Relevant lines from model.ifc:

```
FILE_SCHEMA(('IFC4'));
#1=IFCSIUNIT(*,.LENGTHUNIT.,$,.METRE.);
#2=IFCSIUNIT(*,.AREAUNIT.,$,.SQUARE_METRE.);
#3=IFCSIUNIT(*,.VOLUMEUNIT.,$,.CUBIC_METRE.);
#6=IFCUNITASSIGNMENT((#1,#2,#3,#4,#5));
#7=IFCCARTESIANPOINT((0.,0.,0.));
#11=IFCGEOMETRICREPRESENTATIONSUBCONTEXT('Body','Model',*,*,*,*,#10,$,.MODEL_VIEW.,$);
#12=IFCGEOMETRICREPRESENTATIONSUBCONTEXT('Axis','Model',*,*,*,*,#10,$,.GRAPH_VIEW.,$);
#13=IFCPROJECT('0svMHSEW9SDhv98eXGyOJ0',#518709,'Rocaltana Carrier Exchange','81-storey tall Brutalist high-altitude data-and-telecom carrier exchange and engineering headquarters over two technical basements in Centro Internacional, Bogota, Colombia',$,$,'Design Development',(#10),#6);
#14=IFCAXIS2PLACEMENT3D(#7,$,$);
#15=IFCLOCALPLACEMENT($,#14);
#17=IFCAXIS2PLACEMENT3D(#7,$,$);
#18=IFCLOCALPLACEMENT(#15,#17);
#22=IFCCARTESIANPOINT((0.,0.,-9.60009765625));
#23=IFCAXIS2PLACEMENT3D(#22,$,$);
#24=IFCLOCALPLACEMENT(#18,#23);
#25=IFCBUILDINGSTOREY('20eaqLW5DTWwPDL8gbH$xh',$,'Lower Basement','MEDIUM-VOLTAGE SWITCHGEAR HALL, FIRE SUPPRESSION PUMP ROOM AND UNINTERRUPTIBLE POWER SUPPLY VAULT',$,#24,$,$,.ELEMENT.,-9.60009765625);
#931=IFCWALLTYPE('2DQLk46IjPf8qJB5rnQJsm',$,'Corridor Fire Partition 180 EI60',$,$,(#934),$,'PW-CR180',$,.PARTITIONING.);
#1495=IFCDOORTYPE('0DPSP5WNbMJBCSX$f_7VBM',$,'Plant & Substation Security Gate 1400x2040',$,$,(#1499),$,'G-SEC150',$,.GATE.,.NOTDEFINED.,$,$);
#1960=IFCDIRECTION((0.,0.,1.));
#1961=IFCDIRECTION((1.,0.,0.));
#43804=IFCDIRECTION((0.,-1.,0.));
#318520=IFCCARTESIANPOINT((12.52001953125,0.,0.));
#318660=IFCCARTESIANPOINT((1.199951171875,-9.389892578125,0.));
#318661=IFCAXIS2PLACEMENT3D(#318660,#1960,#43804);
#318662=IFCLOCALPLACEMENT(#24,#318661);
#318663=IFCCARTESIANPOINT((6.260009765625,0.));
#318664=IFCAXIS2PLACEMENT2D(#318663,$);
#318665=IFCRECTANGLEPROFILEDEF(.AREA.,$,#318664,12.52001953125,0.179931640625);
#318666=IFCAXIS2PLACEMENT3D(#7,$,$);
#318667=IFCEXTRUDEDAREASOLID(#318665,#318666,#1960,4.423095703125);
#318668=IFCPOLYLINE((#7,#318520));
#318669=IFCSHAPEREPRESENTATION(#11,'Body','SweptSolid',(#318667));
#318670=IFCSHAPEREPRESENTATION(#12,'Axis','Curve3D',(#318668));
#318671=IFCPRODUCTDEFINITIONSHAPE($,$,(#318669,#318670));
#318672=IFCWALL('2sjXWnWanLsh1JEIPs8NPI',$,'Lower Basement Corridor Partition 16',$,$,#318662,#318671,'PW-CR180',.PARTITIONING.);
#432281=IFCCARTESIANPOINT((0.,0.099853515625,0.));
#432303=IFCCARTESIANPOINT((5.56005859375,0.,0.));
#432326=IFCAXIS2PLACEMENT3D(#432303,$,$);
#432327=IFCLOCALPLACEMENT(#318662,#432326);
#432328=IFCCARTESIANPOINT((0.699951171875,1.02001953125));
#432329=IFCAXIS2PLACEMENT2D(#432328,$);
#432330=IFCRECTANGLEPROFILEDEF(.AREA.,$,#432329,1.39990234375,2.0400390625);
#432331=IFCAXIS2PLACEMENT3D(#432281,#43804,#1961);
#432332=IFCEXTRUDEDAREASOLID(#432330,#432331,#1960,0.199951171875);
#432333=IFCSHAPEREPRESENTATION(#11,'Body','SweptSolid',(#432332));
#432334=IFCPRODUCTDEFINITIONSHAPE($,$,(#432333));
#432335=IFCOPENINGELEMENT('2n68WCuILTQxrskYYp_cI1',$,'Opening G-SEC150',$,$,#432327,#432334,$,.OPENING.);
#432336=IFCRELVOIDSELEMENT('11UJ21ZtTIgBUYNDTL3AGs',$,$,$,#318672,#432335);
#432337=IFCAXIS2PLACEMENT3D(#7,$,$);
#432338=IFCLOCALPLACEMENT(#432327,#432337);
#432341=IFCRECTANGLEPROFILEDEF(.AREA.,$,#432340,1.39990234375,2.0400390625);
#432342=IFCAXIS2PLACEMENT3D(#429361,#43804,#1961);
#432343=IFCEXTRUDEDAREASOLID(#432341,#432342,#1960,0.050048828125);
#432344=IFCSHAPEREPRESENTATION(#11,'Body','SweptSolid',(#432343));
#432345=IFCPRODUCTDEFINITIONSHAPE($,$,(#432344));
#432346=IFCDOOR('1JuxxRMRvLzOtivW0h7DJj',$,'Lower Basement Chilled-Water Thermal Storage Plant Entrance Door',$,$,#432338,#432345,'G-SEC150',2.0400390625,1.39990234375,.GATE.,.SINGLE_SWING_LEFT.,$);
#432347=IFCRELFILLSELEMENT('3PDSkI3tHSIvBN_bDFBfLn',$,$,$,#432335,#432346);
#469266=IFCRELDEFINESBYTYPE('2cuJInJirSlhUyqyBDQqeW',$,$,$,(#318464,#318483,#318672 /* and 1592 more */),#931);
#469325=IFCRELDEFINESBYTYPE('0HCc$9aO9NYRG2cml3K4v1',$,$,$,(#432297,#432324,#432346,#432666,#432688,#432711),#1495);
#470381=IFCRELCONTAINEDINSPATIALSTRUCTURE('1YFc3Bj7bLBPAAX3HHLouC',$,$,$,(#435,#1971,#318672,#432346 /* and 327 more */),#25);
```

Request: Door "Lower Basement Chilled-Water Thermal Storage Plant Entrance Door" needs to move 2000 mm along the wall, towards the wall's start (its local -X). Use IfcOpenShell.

```python
import ifcopenshell
import ifcopenshell.api.geometry
import ifcopenshell.util.placement

model = ifcopenshell.open("model.ifc")

door = model.by_guid("1JuxxRMRvLzOtivW0h7DJj")
opening = door.FillsVoids[0].RelatingOpeningElement
wall = opening.VoidsElements[0].RelatingBuildingElement

wall_matrix = ifcopenshell.util.placement.get_local_placement(wall.ObjectPlacement)
shift = wall_matrix[:3, 0] * -2.0
before = ifcopenshell.util.placement.get_local_placement(door.ObjectPlacement)[:3, 3].copy()

# The door is placed relative to its opening, so it follows when the opening moves.
matrix = ifcopenshell.util.placement.get_local_placement(opening.ObjectPlacement)
matrix[:3, 3] += shift
ifcopenshell.api.geometry.edit_object_placement(
    model, product=opening, matrix=matrix, is_si=False, should_transform_children=True
)

after = ifcopenshell.util.placement.get_local_placement(door.ObjectPlacement)[:3, 3]
print("door moved by", (after - before).round(3) + 0.0)

model.write("model_rev.ifc")
```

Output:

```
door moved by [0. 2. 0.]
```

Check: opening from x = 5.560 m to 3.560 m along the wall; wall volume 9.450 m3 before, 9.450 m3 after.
